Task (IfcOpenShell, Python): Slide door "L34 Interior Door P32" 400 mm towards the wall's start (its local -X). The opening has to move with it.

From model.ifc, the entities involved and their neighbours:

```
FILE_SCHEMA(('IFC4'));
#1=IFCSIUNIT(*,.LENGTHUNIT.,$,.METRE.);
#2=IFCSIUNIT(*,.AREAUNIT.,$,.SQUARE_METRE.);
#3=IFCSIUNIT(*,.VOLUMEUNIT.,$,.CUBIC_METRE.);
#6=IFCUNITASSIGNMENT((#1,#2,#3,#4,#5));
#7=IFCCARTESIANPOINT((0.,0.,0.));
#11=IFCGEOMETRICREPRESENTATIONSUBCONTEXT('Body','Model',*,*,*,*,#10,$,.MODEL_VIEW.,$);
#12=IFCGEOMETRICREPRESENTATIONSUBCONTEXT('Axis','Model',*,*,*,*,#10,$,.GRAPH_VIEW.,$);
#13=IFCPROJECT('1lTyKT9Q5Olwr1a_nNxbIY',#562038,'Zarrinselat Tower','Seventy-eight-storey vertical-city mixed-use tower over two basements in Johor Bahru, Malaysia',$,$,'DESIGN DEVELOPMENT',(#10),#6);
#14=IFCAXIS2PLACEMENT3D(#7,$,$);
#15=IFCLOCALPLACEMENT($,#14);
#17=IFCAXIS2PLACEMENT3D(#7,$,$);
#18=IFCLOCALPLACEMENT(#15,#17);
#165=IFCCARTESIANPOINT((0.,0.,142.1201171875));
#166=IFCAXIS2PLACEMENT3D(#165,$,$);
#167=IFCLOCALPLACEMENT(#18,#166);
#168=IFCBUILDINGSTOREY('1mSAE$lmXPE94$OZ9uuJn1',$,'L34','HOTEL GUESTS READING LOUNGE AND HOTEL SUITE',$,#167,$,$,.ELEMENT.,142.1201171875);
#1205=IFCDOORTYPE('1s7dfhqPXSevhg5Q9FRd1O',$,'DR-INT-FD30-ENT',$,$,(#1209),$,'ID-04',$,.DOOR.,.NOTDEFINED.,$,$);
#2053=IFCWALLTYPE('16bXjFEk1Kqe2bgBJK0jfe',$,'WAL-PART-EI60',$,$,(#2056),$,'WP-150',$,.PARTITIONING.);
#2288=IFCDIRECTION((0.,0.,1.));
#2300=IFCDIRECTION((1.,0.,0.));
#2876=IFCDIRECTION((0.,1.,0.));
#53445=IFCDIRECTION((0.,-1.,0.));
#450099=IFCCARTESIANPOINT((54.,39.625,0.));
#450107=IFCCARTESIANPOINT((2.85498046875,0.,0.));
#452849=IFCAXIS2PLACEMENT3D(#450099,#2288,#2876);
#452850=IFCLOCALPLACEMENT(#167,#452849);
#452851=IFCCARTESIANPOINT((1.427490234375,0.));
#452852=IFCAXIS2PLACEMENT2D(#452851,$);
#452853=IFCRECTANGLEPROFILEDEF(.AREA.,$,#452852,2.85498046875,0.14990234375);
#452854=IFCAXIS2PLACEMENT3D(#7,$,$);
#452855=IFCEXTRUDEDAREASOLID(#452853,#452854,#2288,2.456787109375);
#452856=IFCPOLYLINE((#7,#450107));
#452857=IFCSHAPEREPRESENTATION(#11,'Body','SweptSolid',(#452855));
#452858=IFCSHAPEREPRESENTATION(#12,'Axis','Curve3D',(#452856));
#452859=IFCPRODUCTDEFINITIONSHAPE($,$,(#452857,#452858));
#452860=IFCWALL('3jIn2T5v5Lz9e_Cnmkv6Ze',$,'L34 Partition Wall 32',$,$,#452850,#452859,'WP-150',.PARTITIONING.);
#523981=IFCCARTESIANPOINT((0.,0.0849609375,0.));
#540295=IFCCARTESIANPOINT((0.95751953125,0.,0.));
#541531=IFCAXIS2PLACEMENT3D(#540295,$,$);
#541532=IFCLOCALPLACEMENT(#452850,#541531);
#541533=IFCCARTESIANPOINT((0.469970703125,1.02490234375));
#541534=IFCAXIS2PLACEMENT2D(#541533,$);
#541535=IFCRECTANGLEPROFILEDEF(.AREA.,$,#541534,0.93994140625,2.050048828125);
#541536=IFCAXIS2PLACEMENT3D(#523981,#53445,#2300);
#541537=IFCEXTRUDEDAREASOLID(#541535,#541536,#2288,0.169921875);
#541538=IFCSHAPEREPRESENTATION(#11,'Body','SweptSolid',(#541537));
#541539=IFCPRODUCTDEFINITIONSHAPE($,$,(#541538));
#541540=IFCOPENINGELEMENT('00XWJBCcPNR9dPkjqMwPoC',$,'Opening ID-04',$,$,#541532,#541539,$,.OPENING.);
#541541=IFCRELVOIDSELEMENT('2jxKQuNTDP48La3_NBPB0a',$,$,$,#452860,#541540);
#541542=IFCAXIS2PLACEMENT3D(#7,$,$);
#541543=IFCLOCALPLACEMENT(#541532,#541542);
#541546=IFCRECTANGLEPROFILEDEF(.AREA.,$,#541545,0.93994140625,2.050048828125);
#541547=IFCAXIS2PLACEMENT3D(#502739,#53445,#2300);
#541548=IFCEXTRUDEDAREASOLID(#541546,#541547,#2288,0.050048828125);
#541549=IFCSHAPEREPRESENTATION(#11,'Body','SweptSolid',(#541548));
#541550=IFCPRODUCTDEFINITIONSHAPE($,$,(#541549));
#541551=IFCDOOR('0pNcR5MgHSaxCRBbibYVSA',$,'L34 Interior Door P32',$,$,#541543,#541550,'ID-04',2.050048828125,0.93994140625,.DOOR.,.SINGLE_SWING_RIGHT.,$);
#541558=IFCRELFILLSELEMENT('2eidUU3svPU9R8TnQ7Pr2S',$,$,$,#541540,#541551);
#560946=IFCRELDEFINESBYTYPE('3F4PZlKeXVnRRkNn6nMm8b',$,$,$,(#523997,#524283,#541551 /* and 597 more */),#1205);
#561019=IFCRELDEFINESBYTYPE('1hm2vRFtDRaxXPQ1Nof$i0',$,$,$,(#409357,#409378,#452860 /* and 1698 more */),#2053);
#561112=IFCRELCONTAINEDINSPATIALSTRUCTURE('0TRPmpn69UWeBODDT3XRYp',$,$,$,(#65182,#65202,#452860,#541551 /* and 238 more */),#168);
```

```python
import ifcopenshell
import ifcopenshell.api.geometry
import ifcopenshell.util.placement
import ifcopenshell.util.unit

model = ifcopenshell.open("model.ifc")
unit_scale = ifcopenshell.util.unit.calculate_unit_scale(model)

door = model.by_guid("0pNcR5MgHSaxCRBbibYVSA")
opening = door.FillsVoids[0].RelatingOpeningElement
wall = opening.VoidsElements[0].RelatingBuildingElement

wall_matrix = ifcopenshell.util.placement.get_local_placement(wall.ObjectPlacement)
shift = wall_matrix[:3, 0] * -0.4 / unit_scale
before = ifcopenshell.util.placement.get_local_placement(door.ObjectPlacement)[:3, 3].copy()

# The door is placed relative to its opening, so it follows when the opening moves.
matrix = ifcopenshell.util.placement.get_local_placement(opening.ObjectPlacement)
matrix[:3, 3] += shift
ifcopenshell.api.geometry.edit_object_placement(
    model, product=opening, matrix=matrix, is_si=False, should_transform_children=True
)

after = ifcopenshell.util.placement.get_local_placement(door.ObjectPlacement)[:3, 3]
print("door moved by", (after - before).round(3) + 0.0)

model.write("model-out.ifc")
```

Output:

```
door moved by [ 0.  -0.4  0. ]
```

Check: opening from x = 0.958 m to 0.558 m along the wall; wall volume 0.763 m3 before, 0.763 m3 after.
